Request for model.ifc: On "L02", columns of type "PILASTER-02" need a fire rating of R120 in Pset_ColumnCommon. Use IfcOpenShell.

First a look at what the model holds.

```python
import ifcopenshell
import ifcopenshell.util.element

model = ifcopenshell.open("model.ifc")
print(model.schema)
storey = next(s for s in model.by_type("IfcBuildingStorey") if s.Name == "L02")
columns = [e for e in ifcopenshell.util.element.get_decomposition(storey) if e.is_a("IfcColumn")]
seen = {}
for e in columns:
    element_type = ifcopenshell.util.element.get_type(e)
    key = (element_type.Name if element_type != e and element_type else None, ifcopenshell.util.element.get_pset(e, "Pset_ColumnCommon", "FireRating"))
    seen[key] = seen.get(key, 0) + 1
for (name, value), count in sorted(seen.items(), key=str):
    print(count, "x", name, "|", value)
```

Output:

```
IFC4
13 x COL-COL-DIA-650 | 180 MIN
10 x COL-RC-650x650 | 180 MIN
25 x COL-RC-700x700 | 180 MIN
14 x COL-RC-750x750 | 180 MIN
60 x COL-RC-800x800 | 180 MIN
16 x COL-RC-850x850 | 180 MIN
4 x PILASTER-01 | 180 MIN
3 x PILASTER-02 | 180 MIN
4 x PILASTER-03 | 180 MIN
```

```python
import ifcopenshell
import ifcopenshell.api.pset
import ifcopenshell.util.element

model = ifcopenshell.open("model.ifc")

storey = next(s for s in model.by_type("IfcBuildingStorey") if s.Name == "L02")
columns = [e for e in ifcopenshell.util.element.get_decomposition(storey) if e.is_a("IfcColumn")]

count = 0
for e in columns:
    element_type = ifcopenshell.util.element.get_type(e)
    if element_type in (None, e) or element_type.Name != "PILASTER-02":
        continue
    # add_pset returns the element's existing set when there is one.
    pset = ifcopenshell.api.pset.add_pset(model, product=e, name="Pset_ColumnCommon")
    ifcopenshell.api.pset.edit_pset(model, pset=pset, properties={"FireRating": "R120"})
    count += 1

print(count, "columns updated")

model.write("model_updated.ifc")
```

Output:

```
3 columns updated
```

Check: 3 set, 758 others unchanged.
